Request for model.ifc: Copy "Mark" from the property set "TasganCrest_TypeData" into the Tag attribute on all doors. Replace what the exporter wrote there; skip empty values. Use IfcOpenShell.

First a look at what the model holds.

```python
import ifcopenshell
import ifcopenshell.util.element

model = ifcopenshell.open("model.ifc")
print(model.schema)
doors = model.by_type("IfcDoor")
print(len(doors), "doors")
for e in doors[:8]:
    source = ifcopenshell.util.element.get_pset(e, "TasganCrest_TypeData", "Mark")
    target = e.Tag
    print(e.id(), repr(source), repr(target), sep=" | ")
```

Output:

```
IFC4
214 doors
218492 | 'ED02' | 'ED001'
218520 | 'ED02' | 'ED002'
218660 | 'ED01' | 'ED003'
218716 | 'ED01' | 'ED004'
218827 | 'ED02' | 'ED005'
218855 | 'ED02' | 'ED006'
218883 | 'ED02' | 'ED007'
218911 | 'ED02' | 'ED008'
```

```python
import ifcopenshell
import ifcopenshell.util.element

model = ifcopenshell.open("model.ifc")

count = 0
for e in model.by_type("IfcDoor"):
    value = ifcopenshell.util.element.get_pset(e, "TasganCrest_TypeData", "Mark")
    current = e.Tag
    if not value or not value.strip() or current == value:
        continue
    e.Tag = value
    count += 1

print(count, "doors updated")

model.write("model_updated.ifc")
```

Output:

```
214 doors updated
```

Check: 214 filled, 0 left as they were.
